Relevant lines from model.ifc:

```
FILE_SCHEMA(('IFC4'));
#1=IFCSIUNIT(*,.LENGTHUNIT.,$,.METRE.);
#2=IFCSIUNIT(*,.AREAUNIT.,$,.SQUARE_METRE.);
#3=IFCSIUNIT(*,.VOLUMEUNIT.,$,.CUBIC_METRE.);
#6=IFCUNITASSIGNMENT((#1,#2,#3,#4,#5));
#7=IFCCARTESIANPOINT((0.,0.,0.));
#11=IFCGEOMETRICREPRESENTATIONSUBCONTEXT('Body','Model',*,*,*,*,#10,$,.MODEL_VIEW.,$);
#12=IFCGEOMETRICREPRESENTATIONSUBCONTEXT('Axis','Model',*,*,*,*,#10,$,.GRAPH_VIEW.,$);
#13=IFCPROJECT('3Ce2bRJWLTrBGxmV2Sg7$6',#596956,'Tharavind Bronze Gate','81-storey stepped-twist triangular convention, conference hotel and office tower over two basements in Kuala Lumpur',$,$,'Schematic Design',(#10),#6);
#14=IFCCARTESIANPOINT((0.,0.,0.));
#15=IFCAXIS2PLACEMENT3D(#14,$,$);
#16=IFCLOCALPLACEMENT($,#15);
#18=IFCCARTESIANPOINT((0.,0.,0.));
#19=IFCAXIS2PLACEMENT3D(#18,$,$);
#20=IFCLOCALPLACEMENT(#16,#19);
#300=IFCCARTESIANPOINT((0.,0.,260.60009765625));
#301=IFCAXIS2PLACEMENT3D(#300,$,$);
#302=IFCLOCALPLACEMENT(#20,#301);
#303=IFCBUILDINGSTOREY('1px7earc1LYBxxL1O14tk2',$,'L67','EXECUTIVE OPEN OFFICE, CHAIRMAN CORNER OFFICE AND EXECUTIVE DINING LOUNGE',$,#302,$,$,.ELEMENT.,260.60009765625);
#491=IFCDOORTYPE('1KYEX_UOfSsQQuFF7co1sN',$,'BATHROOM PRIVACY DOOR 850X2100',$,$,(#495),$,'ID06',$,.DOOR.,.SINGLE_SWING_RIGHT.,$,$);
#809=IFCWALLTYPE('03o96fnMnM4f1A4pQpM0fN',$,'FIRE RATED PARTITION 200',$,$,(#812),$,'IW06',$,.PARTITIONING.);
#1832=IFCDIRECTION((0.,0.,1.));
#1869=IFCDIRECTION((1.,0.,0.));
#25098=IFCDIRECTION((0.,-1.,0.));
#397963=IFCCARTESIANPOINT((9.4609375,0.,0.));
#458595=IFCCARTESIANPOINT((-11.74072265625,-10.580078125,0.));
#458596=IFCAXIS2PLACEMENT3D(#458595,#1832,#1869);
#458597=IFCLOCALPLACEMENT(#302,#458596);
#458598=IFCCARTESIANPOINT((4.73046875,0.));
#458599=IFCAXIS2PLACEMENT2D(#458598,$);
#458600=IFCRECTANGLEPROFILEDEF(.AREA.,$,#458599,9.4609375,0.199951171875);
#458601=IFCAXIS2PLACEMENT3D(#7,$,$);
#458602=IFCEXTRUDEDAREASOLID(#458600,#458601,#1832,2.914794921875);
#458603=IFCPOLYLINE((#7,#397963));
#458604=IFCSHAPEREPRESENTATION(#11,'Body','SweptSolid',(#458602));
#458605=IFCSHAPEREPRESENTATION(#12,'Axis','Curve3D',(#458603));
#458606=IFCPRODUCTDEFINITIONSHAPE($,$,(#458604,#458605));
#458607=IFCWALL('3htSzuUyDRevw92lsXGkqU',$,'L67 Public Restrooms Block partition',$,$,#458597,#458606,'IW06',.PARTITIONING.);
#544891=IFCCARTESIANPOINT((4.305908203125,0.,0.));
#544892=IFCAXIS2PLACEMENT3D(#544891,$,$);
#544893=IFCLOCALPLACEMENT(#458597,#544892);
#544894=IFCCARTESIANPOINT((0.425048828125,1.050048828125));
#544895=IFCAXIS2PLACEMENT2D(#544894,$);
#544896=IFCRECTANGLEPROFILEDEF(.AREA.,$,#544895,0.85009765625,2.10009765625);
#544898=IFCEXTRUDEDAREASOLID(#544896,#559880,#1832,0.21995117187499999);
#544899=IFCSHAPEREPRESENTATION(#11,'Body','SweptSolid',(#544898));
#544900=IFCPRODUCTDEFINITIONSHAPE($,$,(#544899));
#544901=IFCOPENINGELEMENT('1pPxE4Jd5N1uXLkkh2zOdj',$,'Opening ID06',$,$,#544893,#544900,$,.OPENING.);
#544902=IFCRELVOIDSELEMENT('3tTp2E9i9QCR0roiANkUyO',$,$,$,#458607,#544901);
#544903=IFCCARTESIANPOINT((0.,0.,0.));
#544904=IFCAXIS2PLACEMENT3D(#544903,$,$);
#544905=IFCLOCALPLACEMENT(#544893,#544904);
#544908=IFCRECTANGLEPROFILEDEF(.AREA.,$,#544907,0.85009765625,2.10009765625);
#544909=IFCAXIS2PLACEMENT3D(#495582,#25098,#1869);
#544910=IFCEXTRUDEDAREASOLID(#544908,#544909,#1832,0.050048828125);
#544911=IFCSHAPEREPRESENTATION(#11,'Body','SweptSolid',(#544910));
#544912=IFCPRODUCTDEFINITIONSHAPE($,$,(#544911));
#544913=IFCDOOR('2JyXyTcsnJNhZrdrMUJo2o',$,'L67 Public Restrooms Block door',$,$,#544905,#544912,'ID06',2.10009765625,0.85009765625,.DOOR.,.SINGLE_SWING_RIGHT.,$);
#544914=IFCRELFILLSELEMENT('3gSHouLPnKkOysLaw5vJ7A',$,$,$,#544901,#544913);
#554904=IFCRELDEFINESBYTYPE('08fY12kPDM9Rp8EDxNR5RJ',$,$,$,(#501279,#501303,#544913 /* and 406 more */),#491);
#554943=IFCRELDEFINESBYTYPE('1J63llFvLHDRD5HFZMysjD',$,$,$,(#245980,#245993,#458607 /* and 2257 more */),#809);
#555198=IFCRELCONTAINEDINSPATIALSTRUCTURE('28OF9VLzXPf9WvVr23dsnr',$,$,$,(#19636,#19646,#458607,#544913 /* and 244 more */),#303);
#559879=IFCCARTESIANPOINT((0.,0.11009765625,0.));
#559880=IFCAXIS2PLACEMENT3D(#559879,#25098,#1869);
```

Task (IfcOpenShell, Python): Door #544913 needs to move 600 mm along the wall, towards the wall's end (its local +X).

```python
import ifcopenshell
import ifcopenshell.api.geometry
import ifcopenshell.util.placement

model = ifcopenshell.open("model.ifc")

door = model.by_id(544913)
opening = door.FillsVoids[0].RelatingOpeningElement
wall = opening.VoidsElements[0].RelatingBuildingElement

wall_matrix = ifcopenshell.util.placement.get_local_placement(wall.ObjectPlacement)
shift = wall_matrix[:3, 0] * 0.6
before = ifcopenshell.util.placement.get_local_placement(door.ObjectPlacement)[:3, 3].copy()

# The door is placed relative to its opening, so it follows when the opening moves.
matrix = ifcopenshell.util.placement.get_local_placement(opening.ObjectPlacement)
matrix[:3, 3] += shift
ifcopenshell.api.geometry.edit_object_placement(
    model, product=opening, matrix=matrix, is_si=False, should_transform_children=True
)

after = ifcopenshell.util.placement.get_local_placement(door.ObjectPlacement)[:3, 3]
print("door moved by", (after - before).round(3) + 0.0)

model.write("model_v2.ifc")
```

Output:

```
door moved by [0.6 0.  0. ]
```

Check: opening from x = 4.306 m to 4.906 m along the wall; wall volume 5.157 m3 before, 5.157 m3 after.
